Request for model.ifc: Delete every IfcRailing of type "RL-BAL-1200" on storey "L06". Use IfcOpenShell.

First a look at what the model holds.

```python
import ifcopenshell
import ifcopenshell.util.element

model = ifcopenshell.open("model.ifc")
print(model.schema)
storey = next(s for s in model.by_type("IfcBuildingStorey") if s.Name == "L06")
railings = [e for e in ifcopenshell.util.element.get_decomposition(storey) if e.is_a("IfcRailing")]
seen = {}
for e in railings:
    element_type = ifcopenshell.util.element.get_type(e)
    name = element_type.Name if element_type not in (None, e) else None
    seen[name] = seen.get(name, 0) + 1
for name, count in sorted(seen.items(), key=str):
    print(count, "x", name)
```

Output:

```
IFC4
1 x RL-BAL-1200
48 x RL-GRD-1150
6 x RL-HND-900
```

```python
import ifcopenshell
import ifcopenshell.api.root
import ifcopenshell.util.element

model = ifcopenshell.open("model.ifc")

storey = next(s for s in model.by_type("IfcBuildingStorey") if s.Name == "L06")
railings = [e for e in ifcopenshell.util.element.get_decomposition(storey) if e.is_a("IfcRailing")]
targets = [e for e in railings if (t := ifcopenshell.util.element.get_type(e)) not in (None, e) and t.Name == "RL-BAL-1200"]

for e in targets:
    ifcopenshell.api.root.remove_product(model, product=e)
print(len(targets), "removed")

model.write("model_rev.ifc")
```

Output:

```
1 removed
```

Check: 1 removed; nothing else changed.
